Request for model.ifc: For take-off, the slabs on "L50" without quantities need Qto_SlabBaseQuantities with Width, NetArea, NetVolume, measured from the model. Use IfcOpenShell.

First a look at what the model holds.

```python
import ifcopenshell
import ifcopenshell.util.element
import ifcopenshell.util.unit

model = ifcopenshell.open("model.ifc")
print(model.schema)
for unit_type in ("LENGTHUNIT", "AREAUNIT", "VOLUMEUNIT"):
    print(unit_type, ifcopenshell.util.unit.calculate_unit_scale(model, unit_type))
storey = next(s for s in model.by_type("IfcBuildingStorey") if s.Name == "L50")
slabs = [e for e in ifcopenshell.util.element.get_decomposition(storey) if e.is_a("IfcSlab")]
for e in sorted(slabs, key=lambda e: e.id()):
    print(e.id(), e.is_a(), e.Name, list(ifcopenshell.util.element.get_psets(e, qtos_only=True)), sep=" | ")
```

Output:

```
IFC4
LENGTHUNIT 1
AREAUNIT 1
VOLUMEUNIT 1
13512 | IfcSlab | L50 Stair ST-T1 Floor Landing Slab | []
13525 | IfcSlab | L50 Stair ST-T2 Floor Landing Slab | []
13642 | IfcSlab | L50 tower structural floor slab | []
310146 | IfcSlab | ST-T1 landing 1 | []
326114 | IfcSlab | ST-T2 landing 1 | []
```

```python
import ifcopenshell
import ifcopenshell.api.pset
import ifcopenshell.geom
import ifcopenshell.util.element
import ifcopenshell.util.shape
import ifcopenshell.util.unit

model = ifcopenshell.open("model.ifc")
unit_scale = ifcopenshell.util.unit.calculate_unit_scale(model)
area_scale = ifcopenshell.util.unit.calculate_unit_scale(model, "AREAUNIT")
volume_scale = ifcopenshell.util.unit.calculate_unit_scale(model, "VOLUMEUNIT")
settings = ifcopenshell.geom.settings()

storey = next(s for s in model.by_type("IfcBuildingStorey") if s.Name == "L50")
slabs = [e for e in ifcopenshell.util.element.get_decomposition(storey) if e.is_a("IfcSlab")]

for e in sorted(slabs, key=lambda e: e.id()):
    if ifcopenshell.util.element.get_psets(e, qtos_only=True, should_inherit=False):
        continue
    # Geometry comes back in metres, in the element's own axes.
    shape = ifcopenshell.geom.create_shape(settings, e)
    values = {
        "Width": ifcopenshell.util.shape.get_z(shape.geometry) / unit_scale,
        "NetArea": ifcopenshell.util.shape.get_footprint_area(shape.geometry) / area_scale,
        "NetVolume": ifcopenshell.util.shape.get_volume(shape.geometry) / volume_scale,
    }
    qto = ifcopenshell.api.pset.add_qto(model, product=e, name="Qto_SlabBaseQuantities")
    ifcopenshell.api.pset.edit_qto(model, qto=qto, properties=values)
    print(e.id(), {k: round(v, 3) for k, v in values.items()})

model.write("model_edited.ifc")
```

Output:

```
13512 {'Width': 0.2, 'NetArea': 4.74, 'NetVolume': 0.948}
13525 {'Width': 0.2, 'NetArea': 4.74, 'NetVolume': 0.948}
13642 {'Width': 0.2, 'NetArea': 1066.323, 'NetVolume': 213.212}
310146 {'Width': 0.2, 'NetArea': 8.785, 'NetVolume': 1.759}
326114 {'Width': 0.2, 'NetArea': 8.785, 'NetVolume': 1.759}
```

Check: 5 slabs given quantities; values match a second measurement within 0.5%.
